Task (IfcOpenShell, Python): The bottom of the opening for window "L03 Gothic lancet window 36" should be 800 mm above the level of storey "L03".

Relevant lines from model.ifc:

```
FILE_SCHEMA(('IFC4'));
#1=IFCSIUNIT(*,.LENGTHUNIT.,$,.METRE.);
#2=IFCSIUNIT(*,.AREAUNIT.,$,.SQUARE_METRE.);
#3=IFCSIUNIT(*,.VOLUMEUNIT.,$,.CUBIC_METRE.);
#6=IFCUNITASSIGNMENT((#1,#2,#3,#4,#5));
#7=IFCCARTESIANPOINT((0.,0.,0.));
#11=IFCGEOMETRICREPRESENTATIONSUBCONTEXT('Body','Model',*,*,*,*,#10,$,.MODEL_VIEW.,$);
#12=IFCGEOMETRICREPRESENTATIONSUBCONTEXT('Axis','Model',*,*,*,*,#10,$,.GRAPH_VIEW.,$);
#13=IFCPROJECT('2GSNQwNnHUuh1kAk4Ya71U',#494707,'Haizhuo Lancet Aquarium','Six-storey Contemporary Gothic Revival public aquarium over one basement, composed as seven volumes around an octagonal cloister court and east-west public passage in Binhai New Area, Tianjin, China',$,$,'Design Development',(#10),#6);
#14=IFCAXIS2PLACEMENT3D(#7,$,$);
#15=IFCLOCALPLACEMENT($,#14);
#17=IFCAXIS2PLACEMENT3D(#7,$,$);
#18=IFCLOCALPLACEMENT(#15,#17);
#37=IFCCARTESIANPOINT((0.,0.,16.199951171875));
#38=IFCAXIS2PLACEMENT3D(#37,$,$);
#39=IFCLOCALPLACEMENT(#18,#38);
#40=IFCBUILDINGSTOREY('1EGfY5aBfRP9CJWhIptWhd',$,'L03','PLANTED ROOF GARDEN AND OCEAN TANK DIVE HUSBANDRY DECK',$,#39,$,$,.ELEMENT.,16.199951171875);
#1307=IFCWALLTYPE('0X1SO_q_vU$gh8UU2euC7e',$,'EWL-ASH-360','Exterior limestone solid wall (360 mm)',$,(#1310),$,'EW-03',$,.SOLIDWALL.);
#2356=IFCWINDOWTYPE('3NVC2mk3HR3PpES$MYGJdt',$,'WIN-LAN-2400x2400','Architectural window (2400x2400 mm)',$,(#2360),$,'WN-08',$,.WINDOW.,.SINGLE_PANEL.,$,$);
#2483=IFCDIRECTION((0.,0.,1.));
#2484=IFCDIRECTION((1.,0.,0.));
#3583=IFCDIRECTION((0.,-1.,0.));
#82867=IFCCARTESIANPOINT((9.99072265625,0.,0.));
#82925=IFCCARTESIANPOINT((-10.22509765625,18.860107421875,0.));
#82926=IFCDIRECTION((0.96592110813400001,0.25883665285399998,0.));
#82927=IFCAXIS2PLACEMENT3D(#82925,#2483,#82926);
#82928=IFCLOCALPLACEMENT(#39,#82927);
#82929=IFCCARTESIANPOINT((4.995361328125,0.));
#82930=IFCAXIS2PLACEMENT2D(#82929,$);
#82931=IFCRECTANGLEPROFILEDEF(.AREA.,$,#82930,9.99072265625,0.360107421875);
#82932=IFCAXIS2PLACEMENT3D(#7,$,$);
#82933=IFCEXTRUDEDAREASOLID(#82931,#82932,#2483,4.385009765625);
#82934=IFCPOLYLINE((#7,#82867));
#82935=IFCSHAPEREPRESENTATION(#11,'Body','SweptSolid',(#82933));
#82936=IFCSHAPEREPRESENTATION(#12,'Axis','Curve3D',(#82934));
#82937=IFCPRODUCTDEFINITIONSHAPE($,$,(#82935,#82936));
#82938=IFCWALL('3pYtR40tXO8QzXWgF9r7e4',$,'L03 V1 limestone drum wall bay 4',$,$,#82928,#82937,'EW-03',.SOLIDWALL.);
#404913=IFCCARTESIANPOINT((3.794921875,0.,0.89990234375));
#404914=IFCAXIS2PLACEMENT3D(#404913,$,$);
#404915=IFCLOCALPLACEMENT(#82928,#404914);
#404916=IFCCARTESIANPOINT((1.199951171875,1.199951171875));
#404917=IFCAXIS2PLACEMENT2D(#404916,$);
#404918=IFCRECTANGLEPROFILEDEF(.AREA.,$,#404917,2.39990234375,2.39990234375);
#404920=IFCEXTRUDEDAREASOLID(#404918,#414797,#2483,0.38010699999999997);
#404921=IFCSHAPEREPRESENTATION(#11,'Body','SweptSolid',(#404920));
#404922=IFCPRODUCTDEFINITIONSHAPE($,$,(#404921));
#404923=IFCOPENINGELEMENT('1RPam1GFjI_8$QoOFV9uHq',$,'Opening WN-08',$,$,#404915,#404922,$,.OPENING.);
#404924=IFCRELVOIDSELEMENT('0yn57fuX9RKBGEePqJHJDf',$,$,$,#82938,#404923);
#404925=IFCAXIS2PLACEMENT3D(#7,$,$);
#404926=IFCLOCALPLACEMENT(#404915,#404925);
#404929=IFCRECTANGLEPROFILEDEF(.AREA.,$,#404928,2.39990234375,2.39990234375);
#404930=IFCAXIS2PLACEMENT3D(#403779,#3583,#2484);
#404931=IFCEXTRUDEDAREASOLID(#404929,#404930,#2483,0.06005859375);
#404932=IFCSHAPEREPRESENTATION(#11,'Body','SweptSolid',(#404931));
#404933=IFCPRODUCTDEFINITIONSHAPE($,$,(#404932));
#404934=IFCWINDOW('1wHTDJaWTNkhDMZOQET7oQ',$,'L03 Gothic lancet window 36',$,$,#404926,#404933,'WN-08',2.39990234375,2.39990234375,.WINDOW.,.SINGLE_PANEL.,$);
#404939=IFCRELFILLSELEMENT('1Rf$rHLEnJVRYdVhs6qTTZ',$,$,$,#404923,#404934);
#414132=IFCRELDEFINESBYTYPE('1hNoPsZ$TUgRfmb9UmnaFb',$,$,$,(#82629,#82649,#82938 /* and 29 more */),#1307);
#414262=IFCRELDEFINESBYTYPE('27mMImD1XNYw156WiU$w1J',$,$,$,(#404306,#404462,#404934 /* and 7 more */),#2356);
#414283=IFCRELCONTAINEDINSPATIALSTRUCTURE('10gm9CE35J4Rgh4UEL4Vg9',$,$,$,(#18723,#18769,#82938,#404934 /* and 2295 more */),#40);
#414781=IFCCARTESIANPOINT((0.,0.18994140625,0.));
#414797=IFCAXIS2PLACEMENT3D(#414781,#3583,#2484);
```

```python
import numpy as np
import ifcopenshell
import ifcopenshell.api.geometry
import ifcopenshell.geom
import ifcopenshell.util.element
import ifcopenshell.util.placement
import ifcopenshell.util.shape
import ifcopenshell.util.unit

model = ifcopenshell.open("model.ifc")
unit_scale = ifcopenshell.util.unit.calculate_unit_scale(model)

window = model.by_guid("1wHTDJaWTNkhDMZOQET7oQ")
opening = window.FillsVoids[0].RelatingOpeningElement
storey = ifcopenshell.util.element.get_container(window, ifc_class="IfcBuildingStorey")
level = ifcopenshell.util.placement.get_local_placement(storey.ObjectPlacement)[2, 3]

# The opening's origin need not be at the sill, so measure its lowest point.
shape = ifcopenshell.geom.create_shape(ifcopenshell.geom.settings(), opening)
bottom = ifcopenshell.util.shape.get_shape_bottom_elevation(shape, shape.geometry) / unit_scale
dz = level + 0.8 / unit_scale - bottom

shift = np.array([0.0, 0.0, dz])
# The window is placed relative to its opening, so it follows when the opening moves.
matrix = ifcopenshell.util.placement.get_local_placement(opening.ObjectPlacement)
matrix[:3, 3] += shift
ifcopenshell.api.geometry.edit_object_placement(
    model, product=opening, matrix=matrix, is_si=False, should_transform_children=True
)

print(f"moved by {dz * unit_scale:+.3f} m")

model.write("model-out.ifc")
```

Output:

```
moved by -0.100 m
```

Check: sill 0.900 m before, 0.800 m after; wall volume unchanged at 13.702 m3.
